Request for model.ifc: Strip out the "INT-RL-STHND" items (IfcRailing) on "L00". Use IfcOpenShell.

First a look at what the model holds.

```python
import ifcopenshell
import ifcopenshell.util.element

model = ifcopenshell.open("model.ifc")
print(model.schema)
storey = next(s for s in model.by_type("IfcBuildingStorey") if s.Name == "L00")
railings = [e for e in ifcopenshell.util.element.get_decomposition(storey) if e.is_a("IfcRailing")]
seen = {}
for e in railings:
    element_type = ifcopenshell.util.element.get_type(e)
    name = element_type.Name if element_type not in (None, e) else None
    seen[name] = seen.get(name, 0) + 1
for name, count in sorted(seen.items(), key=str):
    print(count, "x", name)
```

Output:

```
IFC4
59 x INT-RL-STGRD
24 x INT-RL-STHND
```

```python
import ifcopenshell
import ifcopenshell.api.root
import ifcopenshell.util.element

model = ifcopenshell.open("model.ifc")

storey = next(s for s in model.by_type("IfcBuildingStorey") if s.Name == "L00")
railings = [e for e in ifcopenshell.util.element.get_decomposition(storey) if e.is_a("IfcRailing")]
targets = [e for e in railings if (t := ifcopenshell.util.element.get_type(e)) not in (None, e) and t.Name == "INT-RL-STHND"]

for e in targets:
    ifcopenshell.api.root.remove_product(model, product=e)
print(len(targets), "removed")

model.write("model-out.ifc")
```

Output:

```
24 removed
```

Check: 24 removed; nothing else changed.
